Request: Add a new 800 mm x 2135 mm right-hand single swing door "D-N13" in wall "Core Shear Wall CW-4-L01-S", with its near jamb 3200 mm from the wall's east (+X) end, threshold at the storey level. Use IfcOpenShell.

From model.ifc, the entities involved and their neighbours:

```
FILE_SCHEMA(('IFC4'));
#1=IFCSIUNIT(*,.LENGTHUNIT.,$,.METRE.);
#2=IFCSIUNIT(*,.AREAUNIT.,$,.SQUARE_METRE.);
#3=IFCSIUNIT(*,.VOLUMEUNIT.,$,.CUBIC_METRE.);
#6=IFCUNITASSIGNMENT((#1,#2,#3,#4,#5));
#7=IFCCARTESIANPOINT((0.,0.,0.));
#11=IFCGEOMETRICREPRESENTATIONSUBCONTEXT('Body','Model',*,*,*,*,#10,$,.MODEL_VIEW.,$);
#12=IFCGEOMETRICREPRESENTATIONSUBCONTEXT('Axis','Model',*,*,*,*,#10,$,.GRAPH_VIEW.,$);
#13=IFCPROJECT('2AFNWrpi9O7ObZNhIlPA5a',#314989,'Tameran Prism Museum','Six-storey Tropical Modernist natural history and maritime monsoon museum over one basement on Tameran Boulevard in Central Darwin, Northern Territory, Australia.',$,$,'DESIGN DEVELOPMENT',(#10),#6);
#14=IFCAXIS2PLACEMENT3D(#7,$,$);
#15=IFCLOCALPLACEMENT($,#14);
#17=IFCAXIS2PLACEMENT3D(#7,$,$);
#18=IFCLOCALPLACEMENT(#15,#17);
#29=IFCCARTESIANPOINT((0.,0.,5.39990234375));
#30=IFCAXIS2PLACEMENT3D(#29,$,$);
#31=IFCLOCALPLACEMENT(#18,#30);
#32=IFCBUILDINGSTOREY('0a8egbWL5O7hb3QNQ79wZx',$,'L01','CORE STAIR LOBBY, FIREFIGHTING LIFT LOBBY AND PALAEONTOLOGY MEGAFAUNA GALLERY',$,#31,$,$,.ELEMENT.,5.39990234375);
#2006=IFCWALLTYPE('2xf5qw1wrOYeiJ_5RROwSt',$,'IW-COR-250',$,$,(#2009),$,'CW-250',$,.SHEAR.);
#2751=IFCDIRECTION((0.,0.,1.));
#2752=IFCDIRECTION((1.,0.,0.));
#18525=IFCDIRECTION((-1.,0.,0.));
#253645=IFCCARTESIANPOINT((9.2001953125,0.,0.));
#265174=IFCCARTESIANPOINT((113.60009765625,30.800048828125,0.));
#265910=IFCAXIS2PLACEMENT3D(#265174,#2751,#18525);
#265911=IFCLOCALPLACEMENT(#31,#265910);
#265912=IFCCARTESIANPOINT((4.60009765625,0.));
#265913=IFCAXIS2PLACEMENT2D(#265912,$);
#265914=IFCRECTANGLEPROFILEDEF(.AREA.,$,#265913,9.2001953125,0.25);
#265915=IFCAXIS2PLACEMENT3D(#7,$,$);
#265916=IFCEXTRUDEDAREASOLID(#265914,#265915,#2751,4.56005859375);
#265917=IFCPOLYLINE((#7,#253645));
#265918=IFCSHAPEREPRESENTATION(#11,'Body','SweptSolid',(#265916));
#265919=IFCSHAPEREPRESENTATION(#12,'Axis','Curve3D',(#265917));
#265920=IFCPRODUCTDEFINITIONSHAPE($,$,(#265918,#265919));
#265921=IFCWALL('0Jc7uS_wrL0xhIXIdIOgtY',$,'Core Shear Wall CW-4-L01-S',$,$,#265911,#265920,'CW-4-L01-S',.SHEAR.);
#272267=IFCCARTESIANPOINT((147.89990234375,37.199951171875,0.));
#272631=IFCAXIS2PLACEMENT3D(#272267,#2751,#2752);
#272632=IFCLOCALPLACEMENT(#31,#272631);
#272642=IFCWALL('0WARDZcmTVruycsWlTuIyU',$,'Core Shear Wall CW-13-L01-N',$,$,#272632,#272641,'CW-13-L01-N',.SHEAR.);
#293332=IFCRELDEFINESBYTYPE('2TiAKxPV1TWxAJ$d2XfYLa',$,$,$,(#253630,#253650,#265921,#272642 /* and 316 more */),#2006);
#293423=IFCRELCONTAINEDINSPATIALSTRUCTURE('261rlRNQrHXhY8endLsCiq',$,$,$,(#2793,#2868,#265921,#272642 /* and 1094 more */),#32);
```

```python
import numpy as np
import ifcopenshell
import ifcopenshell.api.feature
import ifcopenshell.api.geometry
import ifcopenshell.api.root
import ifcopenshell.api.spatial
import ifcopenshell.geom
import ifcopenshell.util.element
import ifcopenshell.util.placement
import ifcopenshell.util.representation
import ifcopenshell.util.shape
import ifcopenshell.util.unit

model = ifcopenshell.open("model.ifc")
unit_scale = ifcopenshell.util.unit.calculate_unit_scale(model)
settings = ifcopenshell.geom.settings()


def volume(element):
    """Net volume in cubic metres, openings subtracted."""
    shape = ifcopenshell.geom.create_shape(settings, element)
    return ifcopenshell.util.shape.get_volume(shape.geometry)


wall = model.by_guid("0Jc7uS_wrL0xhIXIdIOgtY")
storey = ifcopenshell.util.element.get_container(wall, ifc_class="IfcBuildingStorey")
context = ifcopenshell.util.representation.get_context(model, "Model", "Body", "MODEL_VIEW")
before = volume(wall)

width, height, from_end, sill = 0.8, 2.135, 3.2, 0.0  # metres

# The wall runs along its own X axis, and the end named is its -X end.
wall_shape = ifcopenshell.geom.create_shape(settings, wall)
x, y, z = ifcopenshell.util.shape.get_vertices(wall_shape.geometry).T
start = x.min() + from_end
face, thickness = float(y.min()), float(y.max() - y.min())
wall_matrix = ifcopenshell.util.placement.get_local_placement(wall.ObjectPlacement)
level = ifcopenshell.util.placement.get_local_placement(storey.ObjectPlacement)[2, 3]


def in_wall(x, y):
    """Placement at x, y metres in the wall's axes, at sill height."""
    matrix = wall_matrix.copy()
    matrix[:, 3] = wall_matrix @ np.array([x / unit_scale, y / unit_scale, 0.0, 1.0])
    matrix[2, 3] = level + sill / unit_scale
    return matrix


# Opening: a box that overshoots both wall faces by 50 mm.
opening = ifcopenshell.api.root.create_entity(model, ifc_class="IfcOpeningElement", predefined_type="OPENING")
box = ifcopenshell.api.geometry.add_wall_representation(
    model, context=context, length=width, height=height, thickness=thickness + 0.1
)
ifcopenshell.api.geometry.assign_representation(model, product=opening, representation=box)
ifcopenshell.api.geometry.edit_object_placement(model, product=opening, matrix=in_wall(start, face - 0.05), is_si=False)
ifcopenshell.api.feature.add_feature(model, feature=opening, element=wall)

door = ifcopenshell.api.root.create_entity(model, ifc_class="IfcDoor", name="D-N13", predefined_type="DOOR")
door.OverallWidth, door.OverallHeight = width / unit_scale, height / unit_scale
door.OperationType = "SINGLE_SWING_RIGHT"
body = ifcopenshell.api.geometry.add_door_representation(
    model,
    context=context,
    overall_width=door.OverallWidth,
    overall_height=door.OverallHeight,
    operation_type="SINGLE_SWING_RIGHT",
    lining_properties={"LiningDepth": thickness / unit_scale, "ThresholdDepth": thickness / unit_scale},
)
ifcopenshell.api.geometry.assign_representation(model, product=door, representation=body)
ifcopenshell.api.spatial.assign_container(model, products=[door], relating_structure=storey)
ifcopenshell.api.feature.add_filling(model, opening=opening, element=door)

# The lining spans the wall, so the door starts at the wall face.
ifcopenshell.api.geometry.edit_object_placement(model, product=door, matrix=in_wall(start, face), is_si=False)

after = volume(wall)

print(f"wall volume {before:.3f} -> {after:.3f} m3")

model.write("model_v2.ifc")
```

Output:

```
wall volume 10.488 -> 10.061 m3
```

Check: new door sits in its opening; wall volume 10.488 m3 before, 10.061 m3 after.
